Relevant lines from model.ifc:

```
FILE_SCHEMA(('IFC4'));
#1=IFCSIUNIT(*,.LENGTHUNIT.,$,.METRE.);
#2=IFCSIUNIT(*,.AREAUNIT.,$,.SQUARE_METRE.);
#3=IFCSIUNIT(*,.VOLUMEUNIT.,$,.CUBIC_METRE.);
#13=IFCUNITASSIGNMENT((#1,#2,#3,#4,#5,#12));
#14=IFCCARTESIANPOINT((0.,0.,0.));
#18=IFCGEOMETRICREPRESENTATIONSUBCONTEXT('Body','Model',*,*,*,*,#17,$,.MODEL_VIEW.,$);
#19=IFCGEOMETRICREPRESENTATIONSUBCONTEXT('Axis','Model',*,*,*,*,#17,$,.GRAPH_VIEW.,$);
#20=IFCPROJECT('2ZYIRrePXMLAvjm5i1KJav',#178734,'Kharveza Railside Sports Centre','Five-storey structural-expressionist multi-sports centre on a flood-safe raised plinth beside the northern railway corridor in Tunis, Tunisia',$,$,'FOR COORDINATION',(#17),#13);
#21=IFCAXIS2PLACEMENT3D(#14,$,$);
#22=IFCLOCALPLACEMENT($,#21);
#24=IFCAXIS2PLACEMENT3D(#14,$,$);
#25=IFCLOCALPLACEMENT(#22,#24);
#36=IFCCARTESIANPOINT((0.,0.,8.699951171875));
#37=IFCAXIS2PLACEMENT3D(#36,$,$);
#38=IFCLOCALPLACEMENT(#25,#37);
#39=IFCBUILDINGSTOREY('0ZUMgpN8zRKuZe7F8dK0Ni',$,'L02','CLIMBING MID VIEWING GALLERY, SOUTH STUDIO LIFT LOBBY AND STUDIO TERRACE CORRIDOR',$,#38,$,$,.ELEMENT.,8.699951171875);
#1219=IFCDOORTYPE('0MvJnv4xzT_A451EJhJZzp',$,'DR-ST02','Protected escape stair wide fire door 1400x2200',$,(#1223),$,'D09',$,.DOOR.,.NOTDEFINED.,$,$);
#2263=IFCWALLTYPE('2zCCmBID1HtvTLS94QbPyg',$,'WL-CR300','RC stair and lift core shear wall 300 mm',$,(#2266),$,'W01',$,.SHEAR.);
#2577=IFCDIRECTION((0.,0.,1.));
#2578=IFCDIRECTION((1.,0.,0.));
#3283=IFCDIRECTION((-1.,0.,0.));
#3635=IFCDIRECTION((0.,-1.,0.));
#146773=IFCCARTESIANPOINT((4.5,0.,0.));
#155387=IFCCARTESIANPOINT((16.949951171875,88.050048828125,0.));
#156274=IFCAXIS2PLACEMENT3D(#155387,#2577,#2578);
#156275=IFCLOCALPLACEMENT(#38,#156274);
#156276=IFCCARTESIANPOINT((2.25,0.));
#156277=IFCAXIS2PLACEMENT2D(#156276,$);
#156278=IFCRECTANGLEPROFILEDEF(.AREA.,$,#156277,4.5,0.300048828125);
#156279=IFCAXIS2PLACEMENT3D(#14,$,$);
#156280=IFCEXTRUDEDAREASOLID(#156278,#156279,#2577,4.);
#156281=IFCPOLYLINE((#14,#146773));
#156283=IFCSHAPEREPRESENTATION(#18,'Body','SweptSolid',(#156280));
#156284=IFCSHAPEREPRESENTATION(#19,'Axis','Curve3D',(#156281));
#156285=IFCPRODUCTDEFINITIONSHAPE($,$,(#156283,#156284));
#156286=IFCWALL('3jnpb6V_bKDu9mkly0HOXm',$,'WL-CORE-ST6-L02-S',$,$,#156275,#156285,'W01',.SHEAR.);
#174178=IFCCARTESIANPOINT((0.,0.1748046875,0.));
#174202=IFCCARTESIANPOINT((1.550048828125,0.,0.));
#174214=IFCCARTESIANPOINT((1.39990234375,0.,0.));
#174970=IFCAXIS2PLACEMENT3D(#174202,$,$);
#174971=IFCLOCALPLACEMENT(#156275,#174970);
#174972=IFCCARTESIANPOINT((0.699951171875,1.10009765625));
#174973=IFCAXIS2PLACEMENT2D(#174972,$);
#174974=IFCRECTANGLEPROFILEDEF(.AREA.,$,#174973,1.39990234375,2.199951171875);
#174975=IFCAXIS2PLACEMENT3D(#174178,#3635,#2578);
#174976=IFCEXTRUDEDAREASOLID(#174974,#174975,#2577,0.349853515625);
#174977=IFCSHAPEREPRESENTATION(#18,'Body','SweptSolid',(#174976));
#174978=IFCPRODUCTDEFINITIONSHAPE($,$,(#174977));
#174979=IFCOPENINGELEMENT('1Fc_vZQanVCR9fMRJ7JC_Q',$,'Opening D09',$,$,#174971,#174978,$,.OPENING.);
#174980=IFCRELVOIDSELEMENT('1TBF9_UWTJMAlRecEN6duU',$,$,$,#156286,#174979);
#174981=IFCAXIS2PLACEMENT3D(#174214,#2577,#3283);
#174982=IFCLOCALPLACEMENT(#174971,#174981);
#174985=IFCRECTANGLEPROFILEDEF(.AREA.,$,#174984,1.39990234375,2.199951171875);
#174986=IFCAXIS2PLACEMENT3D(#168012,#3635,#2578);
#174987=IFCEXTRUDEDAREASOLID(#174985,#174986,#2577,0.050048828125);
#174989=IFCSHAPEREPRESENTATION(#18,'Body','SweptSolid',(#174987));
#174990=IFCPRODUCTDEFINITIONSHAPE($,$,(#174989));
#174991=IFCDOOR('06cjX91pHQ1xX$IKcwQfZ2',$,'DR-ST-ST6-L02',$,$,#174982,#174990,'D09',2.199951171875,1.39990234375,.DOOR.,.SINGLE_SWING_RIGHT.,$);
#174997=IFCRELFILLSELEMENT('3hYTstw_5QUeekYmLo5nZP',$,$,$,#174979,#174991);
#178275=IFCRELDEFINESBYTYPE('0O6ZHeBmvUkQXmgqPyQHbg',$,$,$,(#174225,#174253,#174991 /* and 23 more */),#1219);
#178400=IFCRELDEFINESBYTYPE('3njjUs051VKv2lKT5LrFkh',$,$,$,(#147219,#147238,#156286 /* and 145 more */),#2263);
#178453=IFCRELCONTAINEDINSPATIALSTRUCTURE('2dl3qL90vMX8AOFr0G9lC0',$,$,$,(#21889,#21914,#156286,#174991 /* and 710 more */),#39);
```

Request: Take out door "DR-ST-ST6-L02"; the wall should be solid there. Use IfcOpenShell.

```python
import ifcopenshell
import ifcopenshell.api.feature
import ifcopenshell.api.root
import ifcopenshell.geom
import ifcopenshell.util.shape

model = ifcopenshell.open("model.ifc")
settings = ifcopenshell.geom.settings()


def volume(element):
    """Net volume in cubic metres, openings subtracted."""
    shape = ifcopenshell.geom.create_shape(settings, element)
    return ifcopenshell.util.shape.get_volume(shape.geometry)


door = model.by_guid("06cjX91pHQ1xX$IKcwQfZ2")
opening = door.FillsVoids[0].RelatingOpeningElement
wall = opening.VoidsElements[0].RelatingBuildingElement
before = volume(wall)

ifcopenshell.api.root.remove_product(model, product=door)
ifcopenshell.api.feature.remove_feature(model, feature=opening)

after = volume(wall)

print(f"wall volume {before:.3f} -> {after:.3f} m3")

model.write("model_v2.ifc")
```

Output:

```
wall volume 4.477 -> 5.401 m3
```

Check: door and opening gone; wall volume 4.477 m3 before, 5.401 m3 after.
